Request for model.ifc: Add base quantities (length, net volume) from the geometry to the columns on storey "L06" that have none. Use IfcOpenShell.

First a look at what the model holds.

```python
import ifcopenshell
import ifcopenshell.util.element
import ifcopenshell.util.unit

model = ifcopenshell.open("model.ifc")
print(model.schema)
for unit_type in ("LENGTHUNIT", "AREAUNIT", "VOLUMEUNIT"):
    print(unit_type, ifcopenshell.util.unit.calculate_unit_scale(model, unit_type))
storey = next(s for s in model.by_type("IfcBuildingStorey") if s.Name == "L06")
columns = [e for e in ifcopenshell.util.element.get_decomposition(storey) if e.is_a("IfcColumn")]
for e in sorted(columns, key=lambda e: e.id()):
    print(e.id(), e.is_a(), e.Name, list(ifcopenshell.util.element.get_psets(e, qtos_only=True)), sep=" | ")
```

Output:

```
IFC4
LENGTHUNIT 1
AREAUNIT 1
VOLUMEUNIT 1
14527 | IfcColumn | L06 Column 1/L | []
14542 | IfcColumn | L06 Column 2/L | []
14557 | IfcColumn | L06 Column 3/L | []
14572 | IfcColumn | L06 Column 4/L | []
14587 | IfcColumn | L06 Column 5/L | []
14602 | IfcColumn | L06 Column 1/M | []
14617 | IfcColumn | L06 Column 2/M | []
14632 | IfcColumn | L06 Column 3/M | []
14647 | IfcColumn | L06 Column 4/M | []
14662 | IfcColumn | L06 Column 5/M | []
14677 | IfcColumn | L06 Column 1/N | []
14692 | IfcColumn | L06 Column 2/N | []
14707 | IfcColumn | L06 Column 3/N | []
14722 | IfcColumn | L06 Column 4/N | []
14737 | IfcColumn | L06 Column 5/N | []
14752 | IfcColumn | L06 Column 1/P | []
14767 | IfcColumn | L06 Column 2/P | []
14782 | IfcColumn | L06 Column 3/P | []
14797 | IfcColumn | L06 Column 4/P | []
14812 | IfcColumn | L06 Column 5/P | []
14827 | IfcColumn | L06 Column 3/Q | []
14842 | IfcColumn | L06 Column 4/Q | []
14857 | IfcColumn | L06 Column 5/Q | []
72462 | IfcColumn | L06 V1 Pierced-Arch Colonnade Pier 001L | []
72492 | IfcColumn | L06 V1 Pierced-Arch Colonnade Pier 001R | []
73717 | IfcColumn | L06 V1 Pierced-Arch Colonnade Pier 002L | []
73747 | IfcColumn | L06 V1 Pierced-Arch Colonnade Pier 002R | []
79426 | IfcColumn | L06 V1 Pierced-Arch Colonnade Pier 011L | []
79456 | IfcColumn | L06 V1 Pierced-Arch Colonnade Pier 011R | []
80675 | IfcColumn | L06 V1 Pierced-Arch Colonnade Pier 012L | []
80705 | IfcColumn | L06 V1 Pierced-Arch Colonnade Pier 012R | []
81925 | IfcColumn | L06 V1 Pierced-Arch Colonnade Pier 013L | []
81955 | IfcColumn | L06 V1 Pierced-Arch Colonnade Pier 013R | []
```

```python
import ifcopenshell
import ifcopenshell.api.pset
import ifcopenshell.geom
import ifcopenshell.util.element
import ifcopenshell.util.shape
import ifcopenshell.util.unit

model = ifcopenshell.open("model.ifc")
unit_scale = ifcopenshell.util.unit.calculate_unit_scale(model)
volume_scale = ifcopenshell.util.unit.calculate_unit_scale(model, "VOLUMEUNIT")
settings = ifcopenshell.geom.settings()

storey = next(s for s in model.by_type("IfcBuildingStorey") if s.Name == "L06")
columns = [e for e in ifcopenshell.util.element.get_decomposition(storey) if e.is_a("IfcColumn")]

for e in sorted(columns, key=lambda e: e.id()):
    if ifcopenshell.util.element.get_psets(e, qtos_only=True, should_inherit=False):
        continue
    # Geometry comes back in metres, in the element's own axes.
    shape = ifcopenshell.geom.create_shape(settings, e)
    values = {
        "Length": ifcopenshell.util.shape.get_z(shape.geometry) / unit_scale,
        "NetVolume": ifcopenshell.util.shape.get_volume(shape.geometry) / volume_scale,
    }
    qto = ifcopenshell.api.pset.add_qto(model, product=e, name="Qto_ColumnBaseQuantities")
    ifcopenshell.api.pset.edit_qto(model, qto=qto, properties=values)
    print(e.id(), {k: round(v, 3) for k, v in values.items()})

model.write("model_edited.ifc")
```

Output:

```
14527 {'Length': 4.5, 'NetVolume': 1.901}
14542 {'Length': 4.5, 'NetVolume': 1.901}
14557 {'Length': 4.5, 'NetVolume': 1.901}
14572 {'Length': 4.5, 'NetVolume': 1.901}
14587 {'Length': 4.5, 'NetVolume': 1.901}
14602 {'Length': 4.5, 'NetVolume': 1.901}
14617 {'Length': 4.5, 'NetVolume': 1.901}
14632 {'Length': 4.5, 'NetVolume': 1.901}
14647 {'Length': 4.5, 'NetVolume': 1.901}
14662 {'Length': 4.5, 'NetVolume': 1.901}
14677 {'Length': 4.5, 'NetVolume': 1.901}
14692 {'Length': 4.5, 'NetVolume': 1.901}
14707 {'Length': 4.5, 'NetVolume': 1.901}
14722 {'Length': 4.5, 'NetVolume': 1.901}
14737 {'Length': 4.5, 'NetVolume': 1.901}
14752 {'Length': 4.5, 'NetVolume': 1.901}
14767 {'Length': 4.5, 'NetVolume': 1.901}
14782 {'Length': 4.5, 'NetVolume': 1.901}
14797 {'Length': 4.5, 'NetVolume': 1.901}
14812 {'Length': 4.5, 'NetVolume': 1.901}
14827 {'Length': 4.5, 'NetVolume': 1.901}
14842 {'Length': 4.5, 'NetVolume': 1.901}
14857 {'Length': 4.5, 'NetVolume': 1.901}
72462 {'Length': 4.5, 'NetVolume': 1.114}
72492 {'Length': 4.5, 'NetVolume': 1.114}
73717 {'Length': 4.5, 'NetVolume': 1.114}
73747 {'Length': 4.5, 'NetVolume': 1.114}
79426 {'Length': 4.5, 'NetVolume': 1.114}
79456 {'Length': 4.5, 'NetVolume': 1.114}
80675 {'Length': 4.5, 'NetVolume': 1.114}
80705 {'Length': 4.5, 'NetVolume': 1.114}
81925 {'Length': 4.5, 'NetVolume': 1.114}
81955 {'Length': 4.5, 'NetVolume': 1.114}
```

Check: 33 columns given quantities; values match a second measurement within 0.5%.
